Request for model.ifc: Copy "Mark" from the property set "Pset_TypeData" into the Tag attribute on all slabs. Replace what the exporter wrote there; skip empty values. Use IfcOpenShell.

First a look at what the model holds.

```python
import ifcopenshell
import ifcopenshell.util.element

model = ifcopenshell.open("model.ifc")
print(model.schema)
slabs = model.by_type("IfcSlab")
print(len(slabs), "slabs")
for e in slabs[:8]:
    source = ifcopenshell.util.element.get_pset(e, "Pset_TypeData", "Mark")
    target = e.Tag
    print(e.id(), repr(source), repr(target), sep=" | ")
```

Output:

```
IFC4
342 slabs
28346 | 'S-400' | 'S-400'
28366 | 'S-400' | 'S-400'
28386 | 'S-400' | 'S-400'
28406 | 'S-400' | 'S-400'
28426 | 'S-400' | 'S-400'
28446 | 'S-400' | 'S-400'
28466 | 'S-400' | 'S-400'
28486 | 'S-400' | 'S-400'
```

```python
import ifcopenshell
import ifcopenshell.util.element

model = ifcopenshell.open("model.ifc")

count = 0
for e in model.by_type("IfcSlab"):
    value = ifcopenshell.util.element.get_pset(e, "Pset_TypeData", "Mark")
    current = e.Tag
    if not value or not value.strip() or current == value:
        continue
    e.Tag = value
    count += 1

print(count, "slabs updated")

model.write("model_updated.ifc")
```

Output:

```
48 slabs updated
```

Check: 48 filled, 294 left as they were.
